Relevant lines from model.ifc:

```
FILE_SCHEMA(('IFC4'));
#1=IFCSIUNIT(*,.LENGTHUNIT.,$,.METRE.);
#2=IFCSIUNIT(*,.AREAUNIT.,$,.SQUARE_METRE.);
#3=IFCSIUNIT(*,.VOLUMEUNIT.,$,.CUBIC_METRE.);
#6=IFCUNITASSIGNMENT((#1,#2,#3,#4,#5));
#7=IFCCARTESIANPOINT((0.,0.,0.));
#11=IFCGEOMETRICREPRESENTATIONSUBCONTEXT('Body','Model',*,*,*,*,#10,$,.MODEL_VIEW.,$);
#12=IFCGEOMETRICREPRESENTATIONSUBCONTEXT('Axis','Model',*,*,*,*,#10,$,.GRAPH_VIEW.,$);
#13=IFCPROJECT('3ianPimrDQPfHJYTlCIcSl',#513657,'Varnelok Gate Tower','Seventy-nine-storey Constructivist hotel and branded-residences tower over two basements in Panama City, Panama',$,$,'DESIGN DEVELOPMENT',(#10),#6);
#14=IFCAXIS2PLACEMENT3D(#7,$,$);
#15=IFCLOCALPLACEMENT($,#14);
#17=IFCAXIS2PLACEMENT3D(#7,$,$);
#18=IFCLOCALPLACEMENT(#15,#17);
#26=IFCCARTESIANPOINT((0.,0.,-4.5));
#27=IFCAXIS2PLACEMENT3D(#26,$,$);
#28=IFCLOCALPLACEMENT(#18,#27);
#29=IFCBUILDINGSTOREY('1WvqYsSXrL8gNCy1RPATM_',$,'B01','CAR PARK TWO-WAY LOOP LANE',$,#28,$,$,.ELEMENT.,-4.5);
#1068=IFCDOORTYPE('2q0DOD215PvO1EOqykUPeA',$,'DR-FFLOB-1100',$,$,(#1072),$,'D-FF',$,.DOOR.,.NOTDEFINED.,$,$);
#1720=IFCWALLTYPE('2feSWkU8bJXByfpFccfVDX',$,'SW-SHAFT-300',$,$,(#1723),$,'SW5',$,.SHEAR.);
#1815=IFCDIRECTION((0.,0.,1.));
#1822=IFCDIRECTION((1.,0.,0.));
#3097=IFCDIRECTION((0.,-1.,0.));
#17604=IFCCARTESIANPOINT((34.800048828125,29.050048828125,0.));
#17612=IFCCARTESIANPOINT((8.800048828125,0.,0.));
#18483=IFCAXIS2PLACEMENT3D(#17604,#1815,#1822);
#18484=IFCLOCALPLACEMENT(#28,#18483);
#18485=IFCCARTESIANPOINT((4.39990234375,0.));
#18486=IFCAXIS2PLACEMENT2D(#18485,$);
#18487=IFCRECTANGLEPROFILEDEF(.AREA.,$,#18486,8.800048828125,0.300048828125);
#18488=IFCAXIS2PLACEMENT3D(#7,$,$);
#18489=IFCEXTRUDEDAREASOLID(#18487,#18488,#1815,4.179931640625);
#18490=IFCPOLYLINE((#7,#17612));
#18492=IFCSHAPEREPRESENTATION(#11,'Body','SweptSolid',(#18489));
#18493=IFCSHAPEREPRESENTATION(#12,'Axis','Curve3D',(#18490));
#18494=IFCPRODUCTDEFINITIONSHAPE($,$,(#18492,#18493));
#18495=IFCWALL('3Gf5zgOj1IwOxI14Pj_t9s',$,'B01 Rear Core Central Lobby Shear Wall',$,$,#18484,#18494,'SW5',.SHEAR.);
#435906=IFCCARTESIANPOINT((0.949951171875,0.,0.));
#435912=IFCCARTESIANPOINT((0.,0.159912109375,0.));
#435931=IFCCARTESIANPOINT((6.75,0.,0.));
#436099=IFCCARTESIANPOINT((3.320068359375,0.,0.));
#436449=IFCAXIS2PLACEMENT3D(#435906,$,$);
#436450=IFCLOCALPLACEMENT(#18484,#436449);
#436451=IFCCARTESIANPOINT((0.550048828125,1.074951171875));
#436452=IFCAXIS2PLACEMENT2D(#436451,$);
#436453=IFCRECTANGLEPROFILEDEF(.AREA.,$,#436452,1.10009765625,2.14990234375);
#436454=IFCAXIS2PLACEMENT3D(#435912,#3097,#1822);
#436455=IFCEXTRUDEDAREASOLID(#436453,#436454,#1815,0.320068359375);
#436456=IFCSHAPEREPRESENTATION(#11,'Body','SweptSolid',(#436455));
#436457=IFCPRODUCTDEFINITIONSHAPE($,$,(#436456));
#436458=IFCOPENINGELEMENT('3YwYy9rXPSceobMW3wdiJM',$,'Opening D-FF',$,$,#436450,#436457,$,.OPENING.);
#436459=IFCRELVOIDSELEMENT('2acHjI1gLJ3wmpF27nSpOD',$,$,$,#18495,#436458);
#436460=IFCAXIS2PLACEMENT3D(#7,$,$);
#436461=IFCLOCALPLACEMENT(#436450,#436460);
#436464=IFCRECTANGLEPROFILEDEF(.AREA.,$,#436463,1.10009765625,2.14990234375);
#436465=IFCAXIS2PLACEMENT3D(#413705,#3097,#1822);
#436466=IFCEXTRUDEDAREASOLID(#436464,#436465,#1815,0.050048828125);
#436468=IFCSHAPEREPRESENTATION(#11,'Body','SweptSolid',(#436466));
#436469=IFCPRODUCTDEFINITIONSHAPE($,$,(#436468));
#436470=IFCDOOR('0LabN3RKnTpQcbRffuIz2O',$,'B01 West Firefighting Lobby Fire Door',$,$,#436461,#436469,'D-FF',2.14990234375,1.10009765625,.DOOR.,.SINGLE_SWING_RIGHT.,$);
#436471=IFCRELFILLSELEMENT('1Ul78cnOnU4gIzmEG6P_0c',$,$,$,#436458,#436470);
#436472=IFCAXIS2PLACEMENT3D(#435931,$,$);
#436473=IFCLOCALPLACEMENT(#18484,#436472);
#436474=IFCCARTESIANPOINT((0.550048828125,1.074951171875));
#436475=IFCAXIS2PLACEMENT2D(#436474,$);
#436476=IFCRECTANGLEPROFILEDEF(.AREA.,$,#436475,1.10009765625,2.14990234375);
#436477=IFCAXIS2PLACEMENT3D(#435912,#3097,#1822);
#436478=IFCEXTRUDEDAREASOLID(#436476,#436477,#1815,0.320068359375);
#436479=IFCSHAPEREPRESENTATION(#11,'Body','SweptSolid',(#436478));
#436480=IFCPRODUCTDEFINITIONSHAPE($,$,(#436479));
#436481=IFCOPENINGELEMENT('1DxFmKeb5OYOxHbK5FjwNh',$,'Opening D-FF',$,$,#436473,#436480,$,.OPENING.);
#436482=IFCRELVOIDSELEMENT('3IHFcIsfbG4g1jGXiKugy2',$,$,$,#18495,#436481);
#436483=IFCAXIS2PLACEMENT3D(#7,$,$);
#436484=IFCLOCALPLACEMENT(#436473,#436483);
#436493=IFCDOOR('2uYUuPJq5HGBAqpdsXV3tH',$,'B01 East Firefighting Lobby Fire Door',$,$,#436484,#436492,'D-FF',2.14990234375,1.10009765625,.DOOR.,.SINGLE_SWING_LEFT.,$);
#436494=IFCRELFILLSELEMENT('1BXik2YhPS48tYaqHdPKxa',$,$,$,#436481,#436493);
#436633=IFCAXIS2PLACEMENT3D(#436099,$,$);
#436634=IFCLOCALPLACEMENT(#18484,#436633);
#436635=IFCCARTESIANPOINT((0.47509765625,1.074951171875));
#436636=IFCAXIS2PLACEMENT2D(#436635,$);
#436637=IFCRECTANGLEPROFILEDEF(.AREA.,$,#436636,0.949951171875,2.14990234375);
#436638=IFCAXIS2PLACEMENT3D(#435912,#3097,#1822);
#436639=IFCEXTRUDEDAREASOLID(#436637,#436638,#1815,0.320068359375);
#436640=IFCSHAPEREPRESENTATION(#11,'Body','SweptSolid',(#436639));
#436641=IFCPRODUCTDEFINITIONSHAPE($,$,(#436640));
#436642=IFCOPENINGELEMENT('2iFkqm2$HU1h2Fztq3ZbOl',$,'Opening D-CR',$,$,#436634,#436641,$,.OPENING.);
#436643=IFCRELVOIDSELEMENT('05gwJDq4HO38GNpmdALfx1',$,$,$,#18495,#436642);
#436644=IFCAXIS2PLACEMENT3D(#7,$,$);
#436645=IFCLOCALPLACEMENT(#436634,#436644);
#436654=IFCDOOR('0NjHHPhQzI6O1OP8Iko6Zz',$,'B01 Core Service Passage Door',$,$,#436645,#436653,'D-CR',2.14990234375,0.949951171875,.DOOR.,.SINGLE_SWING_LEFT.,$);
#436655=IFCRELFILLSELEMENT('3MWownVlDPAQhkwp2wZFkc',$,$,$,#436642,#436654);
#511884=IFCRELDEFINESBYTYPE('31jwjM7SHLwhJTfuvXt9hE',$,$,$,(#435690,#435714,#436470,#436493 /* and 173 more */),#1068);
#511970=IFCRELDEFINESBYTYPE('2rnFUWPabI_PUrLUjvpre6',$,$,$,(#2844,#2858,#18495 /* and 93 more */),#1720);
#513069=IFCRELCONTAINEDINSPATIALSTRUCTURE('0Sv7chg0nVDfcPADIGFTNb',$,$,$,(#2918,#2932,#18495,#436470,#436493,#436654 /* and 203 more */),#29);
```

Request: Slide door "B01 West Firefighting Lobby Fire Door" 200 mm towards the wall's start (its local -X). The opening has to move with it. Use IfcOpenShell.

```python
import ifcopenshell
import ifcopenshell.api.geometry
import ifcopenshell.util.placement

model = ifcopenshell.open("model.ifc")

door = model.by_guid("0LabN3RKnTpQcbRffuIz2O")
opening = door.FillsVoids[0].RelatingOpeningElement
wall = opening.VoidsElements[0].RelatingBuildingElement

wall_matrix = ifcopenshell.util.placement.get_local_placement(wall.ObjectPlacement)
shift = wall_matrix[:3, 0] * -0.2
before = ifcopenshell.util.placement.get_local_placement(door.ObjectPlacement)[:3, 3].copy()

# The door is placed relative to its opening, so it follows when the opening moves.
matrix = ifcopenshell.util.placement.get_local_placement(opening.ObjectPlacement)
matrix[:3, 3] += shift
ifcopenshell.api.geometry.edit_object_placement(
    model, product=opening, matrix=matrix, is_si=False, should_transform_children=True
)

after = ifcopenshell.util.placement.get_local_placement(door.ObjectPlacement)[:3, 3]
print("door moved by", (after - before).round(3) + 0.0)

model.write("model-out.ifc")
```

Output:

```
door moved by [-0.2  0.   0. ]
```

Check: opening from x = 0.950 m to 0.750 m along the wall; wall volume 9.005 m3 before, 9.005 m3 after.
